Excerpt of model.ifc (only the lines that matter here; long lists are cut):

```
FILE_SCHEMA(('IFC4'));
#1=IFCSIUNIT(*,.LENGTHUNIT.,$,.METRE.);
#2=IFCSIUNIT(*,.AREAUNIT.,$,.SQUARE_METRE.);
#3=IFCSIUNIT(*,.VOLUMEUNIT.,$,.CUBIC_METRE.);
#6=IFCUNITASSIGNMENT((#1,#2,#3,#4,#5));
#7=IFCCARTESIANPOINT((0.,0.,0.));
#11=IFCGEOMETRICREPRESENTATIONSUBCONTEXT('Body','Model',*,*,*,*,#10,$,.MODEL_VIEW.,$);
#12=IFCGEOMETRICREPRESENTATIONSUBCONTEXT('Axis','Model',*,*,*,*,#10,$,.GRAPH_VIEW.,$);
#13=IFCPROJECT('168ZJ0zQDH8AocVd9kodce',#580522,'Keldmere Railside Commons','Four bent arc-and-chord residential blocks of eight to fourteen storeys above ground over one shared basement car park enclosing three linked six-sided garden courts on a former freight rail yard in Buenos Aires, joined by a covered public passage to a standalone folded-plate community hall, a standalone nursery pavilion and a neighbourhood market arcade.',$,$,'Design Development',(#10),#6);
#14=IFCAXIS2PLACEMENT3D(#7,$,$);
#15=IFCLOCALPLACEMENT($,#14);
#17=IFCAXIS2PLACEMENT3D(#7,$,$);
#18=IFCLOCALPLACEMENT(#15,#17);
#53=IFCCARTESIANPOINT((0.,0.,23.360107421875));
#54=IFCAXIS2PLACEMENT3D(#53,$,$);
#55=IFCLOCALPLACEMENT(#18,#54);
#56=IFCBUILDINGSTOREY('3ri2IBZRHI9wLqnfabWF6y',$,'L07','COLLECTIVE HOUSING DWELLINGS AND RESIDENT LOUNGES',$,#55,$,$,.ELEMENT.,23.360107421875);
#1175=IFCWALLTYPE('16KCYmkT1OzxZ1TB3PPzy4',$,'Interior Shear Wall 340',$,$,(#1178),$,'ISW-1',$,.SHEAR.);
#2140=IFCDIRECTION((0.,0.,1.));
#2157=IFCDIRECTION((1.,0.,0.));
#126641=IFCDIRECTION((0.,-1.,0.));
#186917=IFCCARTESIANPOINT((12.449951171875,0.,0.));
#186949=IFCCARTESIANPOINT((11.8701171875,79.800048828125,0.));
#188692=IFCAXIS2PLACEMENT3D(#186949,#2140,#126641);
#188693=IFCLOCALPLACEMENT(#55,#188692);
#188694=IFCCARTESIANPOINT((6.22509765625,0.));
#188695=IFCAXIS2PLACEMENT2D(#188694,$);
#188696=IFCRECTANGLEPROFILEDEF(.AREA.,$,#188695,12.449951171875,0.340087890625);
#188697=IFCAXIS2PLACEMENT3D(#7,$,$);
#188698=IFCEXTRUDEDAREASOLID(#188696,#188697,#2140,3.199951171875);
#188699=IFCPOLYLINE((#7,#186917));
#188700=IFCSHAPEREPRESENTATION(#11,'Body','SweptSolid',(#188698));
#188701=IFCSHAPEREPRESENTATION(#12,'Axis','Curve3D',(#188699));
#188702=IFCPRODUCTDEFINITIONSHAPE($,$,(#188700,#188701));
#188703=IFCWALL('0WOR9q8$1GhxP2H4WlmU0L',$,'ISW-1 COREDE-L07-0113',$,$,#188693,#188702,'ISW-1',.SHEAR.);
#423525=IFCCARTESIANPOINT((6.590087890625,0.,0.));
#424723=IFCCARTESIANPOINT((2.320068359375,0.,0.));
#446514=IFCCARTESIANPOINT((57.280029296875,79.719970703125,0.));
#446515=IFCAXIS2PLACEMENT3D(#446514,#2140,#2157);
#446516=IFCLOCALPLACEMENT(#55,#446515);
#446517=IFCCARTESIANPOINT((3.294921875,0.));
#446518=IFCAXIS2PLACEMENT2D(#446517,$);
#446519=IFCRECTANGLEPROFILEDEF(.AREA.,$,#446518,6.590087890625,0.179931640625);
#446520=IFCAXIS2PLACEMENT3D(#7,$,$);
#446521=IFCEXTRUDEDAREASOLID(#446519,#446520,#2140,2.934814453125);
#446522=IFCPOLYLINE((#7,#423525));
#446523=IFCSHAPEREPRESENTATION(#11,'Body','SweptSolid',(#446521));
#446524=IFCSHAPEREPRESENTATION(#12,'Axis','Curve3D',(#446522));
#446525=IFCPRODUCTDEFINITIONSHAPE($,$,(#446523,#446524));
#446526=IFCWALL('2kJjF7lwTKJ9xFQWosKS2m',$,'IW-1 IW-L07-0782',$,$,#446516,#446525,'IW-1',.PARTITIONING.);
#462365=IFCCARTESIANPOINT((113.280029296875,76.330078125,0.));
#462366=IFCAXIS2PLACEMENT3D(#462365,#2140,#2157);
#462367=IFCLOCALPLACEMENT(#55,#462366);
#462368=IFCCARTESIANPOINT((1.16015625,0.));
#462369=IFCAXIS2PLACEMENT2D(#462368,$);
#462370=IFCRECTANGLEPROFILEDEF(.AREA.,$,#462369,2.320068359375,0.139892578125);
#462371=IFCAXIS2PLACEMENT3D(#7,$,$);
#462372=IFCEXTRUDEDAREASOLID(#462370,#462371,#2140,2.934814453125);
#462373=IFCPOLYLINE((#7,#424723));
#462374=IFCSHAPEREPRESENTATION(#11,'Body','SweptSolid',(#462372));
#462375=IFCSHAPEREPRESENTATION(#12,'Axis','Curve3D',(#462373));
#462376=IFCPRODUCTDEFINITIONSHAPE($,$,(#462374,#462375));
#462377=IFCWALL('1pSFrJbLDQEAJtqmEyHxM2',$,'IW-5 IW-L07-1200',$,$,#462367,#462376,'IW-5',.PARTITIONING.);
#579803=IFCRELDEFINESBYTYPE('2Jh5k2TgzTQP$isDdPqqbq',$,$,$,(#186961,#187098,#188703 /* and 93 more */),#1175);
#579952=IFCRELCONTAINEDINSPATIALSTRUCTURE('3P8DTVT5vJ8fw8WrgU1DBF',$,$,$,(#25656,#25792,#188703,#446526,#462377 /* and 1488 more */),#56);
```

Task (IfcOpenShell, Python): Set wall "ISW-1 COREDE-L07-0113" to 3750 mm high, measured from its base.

```python
import ifcopenshell
import ifcopenshell.geom
import ifcopenshell.util.representation
import ifcopenshell.util.shape

model = ifcopenshell.open("model.ifc")
settings = ifcopenshell.geom.settings()


def volume(element):
    """Net volume in cubic metres, openings subtracted."""
    shape = ifcopenshell.geom.create_shape(settings, element)
    return ifcopenshell.util.shape.get_volume(shape.geometry)


wall = model.by_guid("0WOR9q8$1GhxP2H4WlmU0L")
before = volume(wall)

body = ifcopenshell.util.representation.get_representation(wall, "Model", "Body")
solid = body.Items[0]
old_height = solid.Depth
solid.Depth = 3.75
after = volume(wall)

print(f"height {old_height:g} -> {solid.Depth:g}, volume {before:.3f} -> {after:.3f} m3")

model.write("model_updated.ifc")
```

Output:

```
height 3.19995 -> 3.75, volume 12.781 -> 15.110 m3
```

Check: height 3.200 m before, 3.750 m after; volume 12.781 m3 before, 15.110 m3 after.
